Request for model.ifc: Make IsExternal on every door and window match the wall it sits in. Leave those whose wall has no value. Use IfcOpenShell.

First a look at what the model holds.

```python
import ifcopenshell
import ifcopenshell.util.element

model = ifcopenshell.open("model.ifc")
print(model.schema)
seen = {}
for e in model.by_type("IfcDoor") + model.by_type("IfcWindow"):
    if not e.FillsVoids:
        continue
    host = e.FillsVoids[0].RelatingOpeningElement.VoidsElements[0].RelatingBuildingElement
    own = ifcopenshell.util.element.get_pset(e, f"Pset_{e.is_a()[3:].removesuffix('StandardCase')}Common", "IsExternal")
    wall = ifcopenshell.util.element.get_pset(host, "Pset_WallCommon", "IsExternal")
    seen[e.is_a(), own, wall] = seen.get((e.is_a(), own, wall), 0) + 1
for (cls, own, wall), count in sorted(seen.items(), key=str):
    print(count, cls, "IsExternal:", own, "| host wall:", wall)
```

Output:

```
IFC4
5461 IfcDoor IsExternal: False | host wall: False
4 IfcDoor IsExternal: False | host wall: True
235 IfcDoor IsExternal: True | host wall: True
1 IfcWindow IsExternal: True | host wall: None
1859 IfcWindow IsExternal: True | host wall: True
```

```python
import ifcopenshell
import ifcopenshell.api.pset
import ifcopenshell.util.element

model = ifcopenshell.open("model.ifc")

count = 0
for ifc_class, pset_name in (("IfcDoor", "Pset_DoorCommon"), ("IfcWindow", "Pset_WindowCommon")):
    for e in model.by_type(ifc_class):
        if not e.FillsVoids:
            continue
        host = e.FillsVoids[0].RelatingOpeningElement.VoidsElements[0].RelatingBuildingElement
        external = ifcopenshell.util.element.get_pset(host, "Pset_WallCommon", "IsExternal")
        if external is None or ifcopenshell.util.element.get_pset(e, pset_name, "IsExternal") == external:
            continue
        found = ifcopenshell.util.element.get_pset(e, pset_name, should_inherit=False)
        if found:
            pset = model.by_id(found["id"])
            if len(ifcopenshell.util.element.get_elements_by_pset(pset)) > 1:
                pset = ifcopenshell.api.pset.unshare_pset(model, products=[e], pset=pset)[0]
        else:
            pset = ifcopenshell.api.pset.add_pset(model, product=e, name=pset_name)
        ifcopenshell.api.pset.edit_pset(model, pset=pset, properties={"IsExternal": external})
        count += 1

print(count, "updated")

model.write("model-out.ifc")
```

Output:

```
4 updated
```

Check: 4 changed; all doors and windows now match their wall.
